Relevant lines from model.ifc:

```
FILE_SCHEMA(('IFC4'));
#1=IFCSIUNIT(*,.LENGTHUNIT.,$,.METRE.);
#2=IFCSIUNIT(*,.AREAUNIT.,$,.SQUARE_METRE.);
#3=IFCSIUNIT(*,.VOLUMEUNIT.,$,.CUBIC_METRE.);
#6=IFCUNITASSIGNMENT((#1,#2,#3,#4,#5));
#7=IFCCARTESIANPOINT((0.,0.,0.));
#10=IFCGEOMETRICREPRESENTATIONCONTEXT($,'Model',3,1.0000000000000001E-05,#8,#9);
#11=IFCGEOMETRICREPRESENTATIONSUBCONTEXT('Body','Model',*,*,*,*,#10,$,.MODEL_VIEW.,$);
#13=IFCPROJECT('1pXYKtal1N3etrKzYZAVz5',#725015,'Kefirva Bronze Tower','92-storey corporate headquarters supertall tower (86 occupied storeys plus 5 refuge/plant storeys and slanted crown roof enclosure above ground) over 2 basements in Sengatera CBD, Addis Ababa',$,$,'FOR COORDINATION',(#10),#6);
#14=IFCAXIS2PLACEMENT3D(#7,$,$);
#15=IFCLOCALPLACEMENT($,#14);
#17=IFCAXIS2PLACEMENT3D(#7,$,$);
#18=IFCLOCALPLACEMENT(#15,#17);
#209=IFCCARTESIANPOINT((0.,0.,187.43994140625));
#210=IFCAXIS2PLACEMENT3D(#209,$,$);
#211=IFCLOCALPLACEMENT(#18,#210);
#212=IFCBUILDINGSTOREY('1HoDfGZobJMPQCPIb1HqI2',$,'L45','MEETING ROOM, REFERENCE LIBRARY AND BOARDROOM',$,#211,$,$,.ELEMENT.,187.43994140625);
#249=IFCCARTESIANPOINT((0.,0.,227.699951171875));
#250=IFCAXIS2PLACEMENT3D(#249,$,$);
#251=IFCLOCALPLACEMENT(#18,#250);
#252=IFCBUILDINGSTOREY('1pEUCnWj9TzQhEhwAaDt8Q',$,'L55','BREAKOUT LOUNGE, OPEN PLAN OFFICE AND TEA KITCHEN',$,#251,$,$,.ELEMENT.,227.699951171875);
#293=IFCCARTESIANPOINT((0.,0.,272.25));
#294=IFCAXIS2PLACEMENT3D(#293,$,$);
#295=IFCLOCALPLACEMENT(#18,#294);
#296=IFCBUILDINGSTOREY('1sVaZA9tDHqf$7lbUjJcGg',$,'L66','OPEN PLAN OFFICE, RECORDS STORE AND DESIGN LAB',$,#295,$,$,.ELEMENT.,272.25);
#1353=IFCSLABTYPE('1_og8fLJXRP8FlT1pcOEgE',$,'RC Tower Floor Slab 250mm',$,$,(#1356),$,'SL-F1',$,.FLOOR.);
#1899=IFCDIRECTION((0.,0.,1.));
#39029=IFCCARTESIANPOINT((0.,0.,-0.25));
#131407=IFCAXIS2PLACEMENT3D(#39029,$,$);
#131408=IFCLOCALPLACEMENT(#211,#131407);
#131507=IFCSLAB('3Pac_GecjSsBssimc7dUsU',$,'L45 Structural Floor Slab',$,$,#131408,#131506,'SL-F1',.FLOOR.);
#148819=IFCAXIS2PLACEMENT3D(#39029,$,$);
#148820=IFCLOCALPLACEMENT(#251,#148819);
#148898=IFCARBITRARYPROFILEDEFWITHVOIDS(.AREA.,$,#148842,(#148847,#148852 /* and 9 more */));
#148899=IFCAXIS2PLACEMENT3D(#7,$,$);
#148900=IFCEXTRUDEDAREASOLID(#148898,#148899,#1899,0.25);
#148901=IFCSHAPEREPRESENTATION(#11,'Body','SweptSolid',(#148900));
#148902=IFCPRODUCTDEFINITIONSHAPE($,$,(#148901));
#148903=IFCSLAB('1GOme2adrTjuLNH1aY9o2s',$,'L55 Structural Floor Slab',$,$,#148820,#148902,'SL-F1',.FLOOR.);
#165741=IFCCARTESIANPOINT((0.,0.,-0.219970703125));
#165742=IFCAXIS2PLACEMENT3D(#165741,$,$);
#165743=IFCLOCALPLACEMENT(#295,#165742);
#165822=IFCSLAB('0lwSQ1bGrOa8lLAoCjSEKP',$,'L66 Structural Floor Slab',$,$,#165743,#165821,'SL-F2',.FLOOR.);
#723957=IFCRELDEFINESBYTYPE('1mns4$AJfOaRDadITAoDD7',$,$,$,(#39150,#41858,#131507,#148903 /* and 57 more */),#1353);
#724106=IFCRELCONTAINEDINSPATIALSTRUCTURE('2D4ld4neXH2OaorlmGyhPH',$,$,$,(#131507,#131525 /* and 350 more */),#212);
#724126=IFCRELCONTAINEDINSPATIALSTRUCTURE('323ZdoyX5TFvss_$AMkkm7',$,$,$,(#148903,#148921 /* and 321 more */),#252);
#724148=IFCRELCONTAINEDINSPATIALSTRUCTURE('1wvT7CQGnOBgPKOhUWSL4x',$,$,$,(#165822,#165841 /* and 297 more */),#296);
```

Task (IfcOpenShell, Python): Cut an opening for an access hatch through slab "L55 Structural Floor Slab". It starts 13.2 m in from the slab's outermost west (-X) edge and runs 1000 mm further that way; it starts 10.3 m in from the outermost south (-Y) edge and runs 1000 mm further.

```python
import numpy as np
import ifcopenshell
import ifcopenshell.api.feature
import ifcopenshell.api.geometry
import ifcopenshell.api.root
import ifcopenshell.geom
import ifcopenshell.util.placement
import ifcopenshell.util.representation
import ifcopenshell.util.shape
import ifcopenshell.util.unit

model = ifcopenshell.open("model.ifc")
unit_scale = ifcopenshell.util.unit.calculate_unit_scale(model)
settings = ifcopenshell.geom.settings()


def volume(element):
    """Net volume in cubic metres, openings subtracted."""
    shape = ifcopenshell.geom.create_shape(settings, element)
    return ifcopenshell.util.shape.get_volume(shape.geometry)


slab = model.by_guid("1GOme2adrTjuLNH1aY9o2s")
before = volume(slab)

# Extent in the slab's own axes, in metres. The edges named are its -X and -Y sides.
slab_shape = ifcopenshell.geom.create_shape(settings, slab)
vertices = ifcopenshell.util.shape.get_vertices(slab_shape.geometry)
x_min, y_min, bottom = vertices.min(axis=0)
top = vertices[:, 2].max()

opening = ifcopenshell.api.root.create_entity(model, ifc_class="IfcOpeningElement", name="Access hatch opening", predefined_type="OPENING")
context = ifcopenshell.util.representation.get_context(model, "Model", "Body", "MODEL_VIEW")
width, depth = 1, 1
outline = [(0.0, 0.0), (width, 0.0), (width, depth), (0.0, depth), (0.0, 0.0)]
# Overshoot both faces by 50 mm so the cut is clean.
shape = ifcopenshell.api.geometry.add_slab_representation(
    model, context=context, depth=top - bottom + 0.1, polyline=outline
)
ifcopenshell.api.geometry.assign_representation(model, product=opening, representation=shape)

matrix = ifcopenshell.util.placement.get_local_placement(slab.ObjectPlacement)
matrix[:, 3] = matrix @ np.append(np.array([x_min + 13.2, y_min + 10.3, bottom - 0.05]) / unit_scale, 1.0)
ifcopenshell.api.geometry.edit_object_placement(model, product=opening, matrix=matrix, is_si=False)
ifcopenshell.api.feature.add_feature(model, feature=opening, element=slab)

after = volume(slab)

print(f"slab volume {before:.3f} -> {after:.3f} m3")

model.write("model_edited.ifc")
```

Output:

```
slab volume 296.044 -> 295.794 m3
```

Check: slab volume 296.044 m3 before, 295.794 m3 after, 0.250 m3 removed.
